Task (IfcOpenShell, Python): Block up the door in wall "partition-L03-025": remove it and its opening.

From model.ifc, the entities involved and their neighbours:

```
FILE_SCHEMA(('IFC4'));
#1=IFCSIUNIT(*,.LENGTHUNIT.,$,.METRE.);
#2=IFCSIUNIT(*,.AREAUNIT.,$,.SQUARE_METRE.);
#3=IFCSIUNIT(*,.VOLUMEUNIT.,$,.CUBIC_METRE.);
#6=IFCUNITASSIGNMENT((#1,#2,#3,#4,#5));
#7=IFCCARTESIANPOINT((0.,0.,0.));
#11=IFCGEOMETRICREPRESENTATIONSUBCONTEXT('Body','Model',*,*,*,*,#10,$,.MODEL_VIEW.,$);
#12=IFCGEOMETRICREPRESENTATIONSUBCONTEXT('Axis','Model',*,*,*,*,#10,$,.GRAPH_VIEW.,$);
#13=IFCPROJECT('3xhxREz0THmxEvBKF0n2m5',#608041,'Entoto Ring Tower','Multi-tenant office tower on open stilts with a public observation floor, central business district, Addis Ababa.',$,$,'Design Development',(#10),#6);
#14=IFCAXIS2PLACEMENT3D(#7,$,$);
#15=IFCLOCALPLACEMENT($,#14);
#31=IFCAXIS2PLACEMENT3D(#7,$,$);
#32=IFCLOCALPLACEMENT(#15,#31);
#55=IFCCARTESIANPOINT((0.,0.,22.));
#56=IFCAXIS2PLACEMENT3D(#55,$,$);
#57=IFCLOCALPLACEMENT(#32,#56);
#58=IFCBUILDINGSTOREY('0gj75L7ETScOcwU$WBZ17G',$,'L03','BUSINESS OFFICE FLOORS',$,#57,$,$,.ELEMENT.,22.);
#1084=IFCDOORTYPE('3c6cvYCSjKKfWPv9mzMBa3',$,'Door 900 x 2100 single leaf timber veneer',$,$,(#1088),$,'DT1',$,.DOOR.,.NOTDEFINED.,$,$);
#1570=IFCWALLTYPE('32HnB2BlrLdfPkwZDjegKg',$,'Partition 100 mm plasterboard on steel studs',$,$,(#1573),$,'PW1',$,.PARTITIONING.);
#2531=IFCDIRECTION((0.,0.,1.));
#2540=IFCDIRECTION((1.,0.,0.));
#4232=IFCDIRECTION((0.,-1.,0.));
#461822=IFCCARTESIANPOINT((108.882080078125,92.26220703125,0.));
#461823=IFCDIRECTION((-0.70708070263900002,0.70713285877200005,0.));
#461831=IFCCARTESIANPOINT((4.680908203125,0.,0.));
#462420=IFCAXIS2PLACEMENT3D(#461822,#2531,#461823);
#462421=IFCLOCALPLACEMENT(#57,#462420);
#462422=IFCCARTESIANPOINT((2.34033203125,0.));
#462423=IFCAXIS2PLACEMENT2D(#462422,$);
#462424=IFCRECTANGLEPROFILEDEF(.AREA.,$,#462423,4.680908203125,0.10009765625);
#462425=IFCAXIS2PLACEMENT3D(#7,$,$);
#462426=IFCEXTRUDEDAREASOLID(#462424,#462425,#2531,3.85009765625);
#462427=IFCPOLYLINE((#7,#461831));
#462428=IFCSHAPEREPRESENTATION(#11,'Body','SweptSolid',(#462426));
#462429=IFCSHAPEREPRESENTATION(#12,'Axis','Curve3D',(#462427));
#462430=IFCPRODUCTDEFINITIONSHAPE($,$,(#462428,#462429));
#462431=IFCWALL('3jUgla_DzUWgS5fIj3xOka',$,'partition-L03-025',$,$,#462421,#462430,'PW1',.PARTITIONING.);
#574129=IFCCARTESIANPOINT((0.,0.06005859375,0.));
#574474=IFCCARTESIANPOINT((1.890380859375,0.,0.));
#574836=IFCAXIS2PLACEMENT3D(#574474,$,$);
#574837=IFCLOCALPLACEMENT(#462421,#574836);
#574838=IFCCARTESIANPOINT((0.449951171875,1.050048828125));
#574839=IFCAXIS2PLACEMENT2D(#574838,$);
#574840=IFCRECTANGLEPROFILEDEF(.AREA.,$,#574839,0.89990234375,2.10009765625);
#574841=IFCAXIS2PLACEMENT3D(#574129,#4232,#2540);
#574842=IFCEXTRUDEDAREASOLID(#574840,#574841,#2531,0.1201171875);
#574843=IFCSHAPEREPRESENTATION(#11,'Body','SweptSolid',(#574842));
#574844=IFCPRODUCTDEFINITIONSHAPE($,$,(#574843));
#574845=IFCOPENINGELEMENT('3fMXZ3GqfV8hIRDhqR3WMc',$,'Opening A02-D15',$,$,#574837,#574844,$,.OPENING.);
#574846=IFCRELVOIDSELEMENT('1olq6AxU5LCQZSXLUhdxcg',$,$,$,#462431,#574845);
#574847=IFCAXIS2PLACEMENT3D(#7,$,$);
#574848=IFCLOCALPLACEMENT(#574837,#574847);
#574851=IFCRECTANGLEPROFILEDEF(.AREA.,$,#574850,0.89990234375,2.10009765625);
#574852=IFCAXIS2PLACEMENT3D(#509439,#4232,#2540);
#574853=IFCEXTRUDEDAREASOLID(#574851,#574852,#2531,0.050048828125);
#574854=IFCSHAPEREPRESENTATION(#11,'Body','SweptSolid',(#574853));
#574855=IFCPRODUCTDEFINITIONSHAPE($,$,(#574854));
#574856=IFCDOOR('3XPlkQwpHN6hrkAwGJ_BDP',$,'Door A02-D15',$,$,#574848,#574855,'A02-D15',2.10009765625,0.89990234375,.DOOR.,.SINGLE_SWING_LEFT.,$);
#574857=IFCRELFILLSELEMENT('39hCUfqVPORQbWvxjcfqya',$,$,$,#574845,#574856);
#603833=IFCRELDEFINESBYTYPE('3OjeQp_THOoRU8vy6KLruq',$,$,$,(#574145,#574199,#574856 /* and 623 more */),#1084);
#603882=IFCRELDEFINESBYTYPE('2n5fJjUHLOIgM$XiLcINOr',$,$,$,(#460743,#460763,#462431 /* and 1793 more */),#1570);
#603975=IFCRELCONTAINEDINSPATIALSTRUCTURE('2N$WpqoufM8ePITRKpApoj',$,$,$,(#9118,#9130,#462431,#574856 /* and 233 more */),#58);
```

```python
import ifcopenshell
import ifcopenshell.api.feature
import ifcopenshell.api.root
import ifcopenshell.geom
import ifcopenshell.util.shape

model = ifcopenshell.open("model.ifc")
settings = ifcopenshell.geom.settings()


def volume(element):
    """Net volume in cubic metres, openings subtracted."""
    shape = ifcopenshell.geom.create_shape(settings, element)
    return ifcopenshell.util.shape.get_volume(shape.geometry)


door = model.by_id(574856)
opening = door.FillsVoids[0].RelatingOpeningElement
wall = opening.VoidsElements[0].RelatingBuildingElement
before = volume(wall)

ifcopenshell.api.root.remove_product(model, product=door)
ifcopenshell.api.feature.remove_feature(model, feature=opening)

after = volume(wall)

print(f"wall volume {before:.3f} -> {after:.3f} m3")

model.write("model_v2.ifc")
```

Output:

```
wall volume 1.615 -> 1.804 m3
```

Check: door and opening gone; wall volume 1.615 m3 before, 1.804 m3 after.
